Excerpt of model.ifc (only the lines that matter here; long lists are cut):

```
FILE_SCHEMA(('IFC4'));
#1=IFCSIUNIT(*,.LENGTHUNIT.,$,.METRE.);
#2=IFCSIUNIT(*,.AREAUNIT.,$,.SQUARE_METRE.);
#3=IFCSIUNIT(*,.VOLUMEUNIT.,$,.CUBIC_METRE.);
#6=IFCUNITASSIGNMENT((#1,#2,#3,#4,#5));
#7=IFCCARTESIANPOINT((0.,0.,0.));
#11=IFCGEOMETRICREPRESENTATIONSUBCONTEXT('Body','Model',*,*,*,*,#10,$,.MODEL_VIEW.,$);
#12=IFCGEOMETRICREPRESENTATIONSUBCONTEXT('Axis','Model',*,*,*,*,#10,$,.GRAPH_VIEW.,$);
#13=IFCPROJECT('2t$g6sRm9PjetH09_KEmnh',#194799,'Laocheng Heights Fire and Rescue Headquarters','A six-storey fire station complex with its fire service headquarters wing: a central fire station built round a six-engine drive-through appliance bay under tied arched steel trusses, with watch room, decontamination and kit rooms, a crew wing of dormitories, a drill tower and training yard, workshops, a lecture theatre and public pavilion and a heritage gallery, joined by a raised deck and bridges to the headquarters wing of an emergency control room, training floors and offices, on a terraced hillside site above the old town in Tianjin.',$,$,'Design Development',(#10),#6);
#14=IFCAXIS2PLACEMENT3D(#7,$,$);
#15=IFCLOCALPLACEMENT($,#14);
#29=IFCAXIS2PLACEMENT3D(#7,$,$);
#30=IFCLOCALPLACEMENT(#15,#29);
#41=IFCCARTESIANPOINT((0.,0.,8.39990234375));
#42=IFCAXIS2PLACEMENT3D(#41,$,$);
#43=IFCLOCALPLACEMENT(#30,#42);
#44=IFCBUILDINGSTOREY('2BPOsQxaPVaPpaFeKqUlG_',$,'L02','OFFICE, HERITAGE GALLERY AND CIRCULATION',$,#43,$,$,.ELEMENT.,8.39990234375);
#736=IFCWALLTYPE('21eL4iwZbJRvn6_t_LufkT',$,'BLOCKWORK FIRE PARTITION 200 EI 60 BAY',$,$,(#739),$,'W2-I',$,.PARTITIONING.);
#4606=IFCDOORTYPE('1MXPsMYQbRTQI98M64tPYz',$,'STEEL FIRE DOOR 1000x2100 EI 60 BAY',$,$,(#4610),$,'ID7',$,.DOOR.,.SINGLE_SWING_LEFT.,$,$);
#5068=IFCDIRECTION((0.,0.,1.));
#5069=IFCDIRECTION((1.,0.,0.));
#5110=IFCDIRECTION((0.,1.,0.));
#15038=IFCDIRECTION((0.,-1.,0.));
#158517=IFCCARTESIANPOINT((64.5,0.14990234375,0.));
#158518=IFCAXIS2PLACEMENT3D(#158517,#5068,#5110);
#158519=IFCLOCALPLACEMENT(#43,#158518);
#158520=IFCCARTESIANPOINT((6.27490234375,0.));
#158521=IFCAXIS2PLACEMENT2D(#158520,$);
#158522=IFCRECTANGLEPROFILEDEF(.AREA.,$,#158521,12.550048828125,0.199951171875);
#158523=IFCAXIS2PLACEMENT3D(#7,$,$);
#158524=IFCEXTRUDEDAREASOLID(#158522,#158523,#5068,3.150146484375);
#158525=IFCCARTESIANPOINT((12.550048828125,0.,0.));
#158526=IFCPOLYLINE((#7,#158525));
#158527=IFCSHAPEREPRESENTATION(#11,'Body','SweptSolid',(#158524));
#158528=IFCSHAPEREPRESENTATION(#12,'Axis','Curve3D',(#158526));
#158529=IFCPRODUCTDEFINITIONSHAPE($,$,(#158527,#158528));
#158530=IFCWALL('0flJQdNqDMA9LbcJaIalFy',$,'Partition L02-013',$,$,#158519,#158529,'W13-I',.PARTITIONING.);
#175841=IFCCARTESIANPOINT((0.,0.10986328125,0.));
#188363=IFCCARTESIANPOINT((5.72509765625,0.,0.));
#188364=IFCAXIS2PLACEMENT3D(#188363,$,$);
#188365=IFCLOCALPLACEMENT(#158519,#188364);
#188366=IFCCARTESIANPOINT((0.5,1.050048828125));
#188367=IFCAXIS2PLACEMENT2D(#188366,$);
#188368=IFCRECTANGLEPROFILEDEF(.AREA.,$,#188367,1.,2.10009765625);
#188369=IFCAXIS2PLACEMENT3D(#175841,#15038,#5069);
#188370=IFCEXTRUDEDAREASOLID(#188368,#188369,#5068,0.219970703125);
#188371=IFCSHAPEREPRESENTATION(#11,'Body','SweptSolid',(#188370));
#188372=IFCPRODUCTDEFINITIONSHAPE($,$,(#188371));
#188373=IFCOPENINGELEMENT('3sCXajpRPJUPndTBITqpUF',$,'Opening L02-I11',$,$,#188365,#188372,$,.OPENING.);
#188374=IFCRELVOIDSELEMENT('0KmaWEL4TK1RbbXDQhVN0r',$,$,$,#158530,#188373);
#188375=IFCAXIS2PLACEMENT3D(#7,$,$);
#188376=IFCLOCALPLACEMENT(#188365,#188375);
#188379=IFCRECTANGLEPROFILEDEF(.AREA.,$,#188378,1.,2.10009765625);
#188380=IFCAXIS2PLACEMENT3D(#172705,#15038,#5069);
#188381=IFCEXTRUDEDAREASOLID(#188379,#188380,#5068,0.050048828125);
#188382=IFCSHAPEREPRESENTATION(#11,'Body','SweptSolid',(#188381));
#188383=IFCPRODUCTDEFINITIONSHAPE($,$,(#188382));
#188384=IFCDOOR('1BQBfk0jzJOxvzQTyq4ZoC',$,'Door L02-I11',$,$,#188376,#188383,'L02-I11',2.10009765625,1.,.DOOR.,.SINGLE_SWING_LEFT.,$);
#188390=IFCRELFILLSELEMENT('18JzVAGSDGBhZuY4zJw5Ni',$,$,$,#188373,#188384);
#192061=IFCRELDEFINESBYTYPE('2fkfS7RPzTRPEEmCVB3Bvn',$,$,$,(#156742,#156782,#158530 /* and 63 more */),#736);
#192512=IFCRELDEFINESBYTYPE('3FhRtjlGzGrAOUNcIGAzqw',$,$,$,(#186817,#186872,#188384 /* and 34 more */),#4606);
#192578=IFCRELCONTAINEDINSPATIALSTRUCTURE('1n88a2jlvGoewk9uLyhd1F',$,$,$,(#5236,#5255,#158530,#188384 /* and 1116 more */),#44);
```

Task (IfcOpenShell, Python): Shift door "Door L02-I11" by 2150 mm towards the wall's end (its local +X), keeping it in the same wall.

```python
import ifcopenshell
import ifcopenshell.api.geometry
import ifcopenshell.util.placement

model = ifcopenshell.open("model.ifc")

door = model.by_id(188384)
opening = door.FillsVoids[0].RelatingOpeningElement
wall = opening.VoidsElements[0].RelatingBuildingElement

wall_matrix = ifcopenshell.util.placement.get_local_placement(wall.ObjectPlacement)
shift = wall_matrix[:3, 0] * 2.15
before = ifcopenshell.util.placement.get_local_placement(door.ObjectPlacement)[:3, 3].copy()

# The door is placed relative to its opening, so it follows when the opening moves.
matrix = ifcopenshell.util.placement.get_local_placement(opening.ObjectPlacement)
matrix[:3, 3] += shift
ifcopenshell.api.geometry.edit_object_placement(
    model, product=opening, matrix=matrix, is_si=False, should_transform_children=True
)

after = ifcopenshell.util.placement.get_local_placement(door.ObjectPlacement)[:3, 3]
print("door moved by", (after - before).round(3) + 0.0)

model.write("model_edited.ifc")
```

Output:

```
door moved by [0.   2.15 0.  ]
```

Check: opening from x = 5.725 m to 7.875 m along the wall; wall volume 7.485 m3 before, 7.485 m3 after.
